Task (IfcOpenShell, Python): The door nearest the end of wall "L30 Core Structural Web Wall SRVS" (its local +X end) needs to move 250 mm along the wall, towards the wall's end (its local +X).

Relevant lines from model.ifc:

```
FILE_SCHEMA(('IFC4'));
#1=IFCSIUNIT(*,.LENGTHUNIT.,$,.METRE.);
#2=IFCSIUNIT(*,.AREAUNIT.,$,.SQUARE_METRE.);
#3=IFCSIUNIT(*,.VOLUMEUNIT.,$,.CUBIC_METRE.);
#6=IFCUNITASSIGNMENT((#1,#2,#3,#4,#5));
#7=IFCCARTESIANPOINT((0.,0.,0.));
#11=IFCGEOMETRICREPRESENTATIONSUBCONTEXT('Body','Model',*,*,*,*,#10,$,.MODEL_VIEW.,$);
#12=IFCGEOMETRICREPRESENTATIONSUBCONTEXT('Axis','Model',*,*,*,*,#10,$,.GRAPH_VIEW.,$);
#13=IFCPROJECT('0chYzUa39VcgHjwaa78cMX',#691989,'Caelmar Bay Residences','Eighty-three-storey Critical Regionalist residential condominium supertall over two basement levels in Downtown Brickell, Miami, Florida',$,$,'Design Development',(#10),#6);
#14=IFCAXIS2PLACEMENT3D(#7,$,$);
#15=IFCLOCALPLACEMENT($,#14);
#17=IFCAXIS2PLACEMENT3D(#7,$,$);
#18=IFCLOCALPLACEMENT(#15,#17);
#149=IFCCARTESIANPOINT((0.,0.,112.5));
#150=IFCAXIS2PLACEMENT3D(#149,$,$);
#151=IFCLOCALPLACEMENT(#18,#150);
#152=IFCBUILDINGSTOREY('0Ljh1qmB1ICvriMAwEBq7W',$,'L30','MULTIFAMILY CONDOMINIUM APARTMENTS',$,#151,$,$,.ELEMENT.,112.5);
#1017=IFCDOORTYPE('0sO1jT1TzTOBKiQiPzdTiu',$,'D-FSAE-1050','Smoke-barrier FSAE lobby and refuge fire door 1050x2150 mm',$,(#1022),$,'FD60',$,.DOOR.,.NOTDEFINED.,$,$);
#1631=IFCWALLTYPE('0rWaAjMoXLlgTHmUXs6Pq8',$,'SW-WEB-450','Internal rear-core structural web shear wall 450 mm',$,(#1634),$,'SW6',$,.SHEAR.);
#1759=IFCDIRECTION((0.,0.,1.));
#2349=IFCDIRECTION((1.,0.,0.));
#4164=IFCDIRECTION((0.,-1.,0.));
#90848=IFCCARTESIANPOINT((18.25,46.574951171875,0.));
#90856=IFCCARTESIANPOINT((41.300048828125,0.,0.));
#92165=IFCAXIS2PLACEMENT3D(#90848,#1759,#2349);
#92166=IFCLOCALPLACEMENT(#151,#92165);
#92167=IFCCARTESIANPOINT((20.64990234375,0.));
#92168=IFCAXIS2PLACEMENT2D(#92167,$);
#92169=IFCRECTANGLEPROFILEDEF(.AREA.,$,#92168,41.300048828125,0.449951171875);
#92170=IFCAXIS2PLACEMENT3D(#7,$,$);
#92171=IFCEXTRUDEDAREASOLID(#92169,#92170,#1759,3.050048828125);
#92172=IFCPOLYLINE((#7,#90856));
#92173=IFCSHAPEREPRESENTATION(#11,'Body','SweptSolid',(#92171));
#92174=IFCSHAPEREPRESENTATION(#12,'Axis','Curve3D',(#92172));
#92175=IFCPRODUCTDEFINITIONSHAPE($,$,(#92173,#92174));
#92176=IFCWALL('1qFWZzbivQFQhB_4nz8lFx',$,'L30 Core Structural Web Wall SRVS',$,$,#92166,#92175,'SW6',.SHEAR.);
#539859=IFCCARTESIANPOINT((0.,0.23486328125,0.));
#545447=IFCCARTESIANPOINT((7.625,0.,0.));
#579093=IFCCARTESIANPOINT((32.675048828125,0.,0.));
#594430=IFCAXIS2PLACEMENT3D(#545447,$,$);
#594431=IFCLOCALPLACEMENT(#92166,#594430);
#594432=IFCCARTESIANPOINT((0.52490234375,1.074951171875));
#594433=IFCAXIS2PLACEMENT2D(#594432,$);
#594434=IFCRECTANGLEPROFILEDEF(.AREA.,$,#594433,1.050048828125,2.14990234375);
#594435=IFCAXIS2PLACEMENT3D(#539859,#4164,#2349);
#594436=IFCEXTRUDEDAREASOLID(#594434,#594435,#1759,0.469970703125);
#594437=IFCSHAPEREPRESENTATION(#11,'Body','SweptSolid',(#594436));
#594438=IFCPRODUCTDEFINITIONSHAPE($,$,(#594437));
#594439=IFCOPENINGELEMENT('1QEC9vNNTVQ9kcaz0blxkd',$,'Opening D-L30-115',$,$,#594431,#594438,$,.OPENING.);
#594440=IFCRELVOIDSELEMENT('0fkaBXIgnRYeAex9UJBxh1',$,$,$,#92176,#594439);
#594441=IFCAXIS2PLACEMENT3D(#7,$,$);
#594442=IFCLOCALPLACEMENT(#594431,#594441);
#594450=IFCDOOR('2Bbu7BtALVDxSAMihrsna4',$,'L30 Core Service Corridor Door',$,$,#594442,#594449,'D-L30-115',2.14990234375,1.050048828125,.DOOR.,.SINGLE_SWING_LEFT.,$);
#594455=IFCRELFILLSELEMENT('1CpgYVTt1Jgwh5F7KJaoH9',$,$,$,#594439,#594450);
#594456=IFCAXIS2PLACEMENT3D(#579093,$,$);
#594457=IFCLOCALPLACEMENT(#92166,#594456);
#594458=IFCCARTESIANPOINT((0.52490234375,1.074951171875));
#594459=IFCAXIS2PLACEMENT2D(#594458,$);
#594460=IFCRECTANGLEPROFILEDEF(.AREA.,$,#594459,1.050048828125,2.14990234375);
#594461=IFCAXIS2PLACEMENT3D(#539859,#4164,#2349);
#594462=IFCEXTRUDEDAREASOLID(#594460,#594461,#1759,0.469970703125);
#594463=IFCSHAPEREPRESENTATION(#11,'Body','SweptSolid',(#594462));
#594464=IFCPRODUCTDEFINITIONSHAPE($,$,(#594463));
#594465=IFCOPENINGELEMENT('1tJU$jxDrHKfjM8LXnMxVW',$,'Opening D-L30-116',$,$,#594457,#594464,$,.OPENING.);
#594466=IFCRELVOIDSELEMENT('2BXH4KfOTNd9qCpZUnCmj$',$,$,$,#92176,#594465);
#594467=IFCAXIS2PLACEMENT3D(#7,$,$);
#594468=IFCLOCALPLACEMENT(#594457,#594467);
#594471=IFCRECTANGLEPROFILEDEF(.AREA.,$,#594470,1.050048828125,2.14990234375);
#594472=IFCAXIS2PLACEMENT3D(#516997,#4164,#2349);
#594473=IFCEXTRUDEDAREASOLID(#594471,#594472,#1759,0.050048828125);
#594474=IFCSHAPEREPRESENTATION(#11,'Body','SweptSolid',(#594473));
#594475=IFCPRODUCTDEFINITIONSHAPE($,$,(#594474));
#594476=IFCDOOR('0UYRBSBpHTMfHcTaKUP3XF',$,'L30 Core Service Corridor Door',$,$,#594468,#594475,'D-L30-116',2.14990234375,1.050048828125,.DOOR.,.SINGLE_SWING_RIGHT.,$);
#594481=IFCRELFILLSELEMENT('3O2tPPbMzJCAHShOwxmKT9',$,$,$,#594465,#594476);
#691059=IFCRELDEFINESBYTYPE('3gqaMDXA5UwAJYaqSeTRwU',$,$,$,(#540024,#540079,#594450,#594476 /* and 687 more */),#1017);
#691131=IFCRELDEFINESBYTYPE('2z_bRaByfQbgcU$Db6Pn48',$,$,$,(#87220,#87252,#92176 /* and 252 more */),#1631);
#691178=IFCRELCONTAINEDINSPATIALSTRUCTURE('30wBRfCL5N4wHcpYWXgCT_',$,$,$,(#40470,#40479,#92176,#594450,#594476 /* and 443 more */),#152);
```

```python
import ifcopenshell
import ifcopenshell.api.geometry
import ifcopenshell.util.placement
import ifcopenshell.util.unit

model = ifcopenshell.open("model.ifc")
unit_scale = ifcopenshell.util.unit.calculate_unit_scale(model)

door = model.by_guid("0UYRBSBpHTMfHcTaKUP3XF")
opening = door.FillsVoids[0].RelatingOpeningElement
wall = opening.VoidsElements[0].RelatingBuildingElement

wall_matrix = ifcopenshell.util.placement.get_local_placement(wall.ObjectPlacement)
shift = wall_matrix[:3, 0] * 0.25 / unit_scale
before = ifcopenshell.util.placement.get_local_placement(door.ObjectPlacement)[:3, 3].copy()

# The door is placed relative to its opening, so it follows when the opening moves.
matrix = ifcopenshell.util.placement.get_local_placement(opening.ObjectPlacement)
matrix[:3, 3] += shift
ifcopenshell.api.geometry.edit_object_placement(
    model, product=opening, matrix=matrix, is_si=False, should_transform_children=True
)

after = ifcopenshell.util.placement.get_local_placement(door.ObjectPlacement)[:3, 3]
print("door moved by", (after - before).round(3) + 0.0)

model.write("model-out.ifc")
```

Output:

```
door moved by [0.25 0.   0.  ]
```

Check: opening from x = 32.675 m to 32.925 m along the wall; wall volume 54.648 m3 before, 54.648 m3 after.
